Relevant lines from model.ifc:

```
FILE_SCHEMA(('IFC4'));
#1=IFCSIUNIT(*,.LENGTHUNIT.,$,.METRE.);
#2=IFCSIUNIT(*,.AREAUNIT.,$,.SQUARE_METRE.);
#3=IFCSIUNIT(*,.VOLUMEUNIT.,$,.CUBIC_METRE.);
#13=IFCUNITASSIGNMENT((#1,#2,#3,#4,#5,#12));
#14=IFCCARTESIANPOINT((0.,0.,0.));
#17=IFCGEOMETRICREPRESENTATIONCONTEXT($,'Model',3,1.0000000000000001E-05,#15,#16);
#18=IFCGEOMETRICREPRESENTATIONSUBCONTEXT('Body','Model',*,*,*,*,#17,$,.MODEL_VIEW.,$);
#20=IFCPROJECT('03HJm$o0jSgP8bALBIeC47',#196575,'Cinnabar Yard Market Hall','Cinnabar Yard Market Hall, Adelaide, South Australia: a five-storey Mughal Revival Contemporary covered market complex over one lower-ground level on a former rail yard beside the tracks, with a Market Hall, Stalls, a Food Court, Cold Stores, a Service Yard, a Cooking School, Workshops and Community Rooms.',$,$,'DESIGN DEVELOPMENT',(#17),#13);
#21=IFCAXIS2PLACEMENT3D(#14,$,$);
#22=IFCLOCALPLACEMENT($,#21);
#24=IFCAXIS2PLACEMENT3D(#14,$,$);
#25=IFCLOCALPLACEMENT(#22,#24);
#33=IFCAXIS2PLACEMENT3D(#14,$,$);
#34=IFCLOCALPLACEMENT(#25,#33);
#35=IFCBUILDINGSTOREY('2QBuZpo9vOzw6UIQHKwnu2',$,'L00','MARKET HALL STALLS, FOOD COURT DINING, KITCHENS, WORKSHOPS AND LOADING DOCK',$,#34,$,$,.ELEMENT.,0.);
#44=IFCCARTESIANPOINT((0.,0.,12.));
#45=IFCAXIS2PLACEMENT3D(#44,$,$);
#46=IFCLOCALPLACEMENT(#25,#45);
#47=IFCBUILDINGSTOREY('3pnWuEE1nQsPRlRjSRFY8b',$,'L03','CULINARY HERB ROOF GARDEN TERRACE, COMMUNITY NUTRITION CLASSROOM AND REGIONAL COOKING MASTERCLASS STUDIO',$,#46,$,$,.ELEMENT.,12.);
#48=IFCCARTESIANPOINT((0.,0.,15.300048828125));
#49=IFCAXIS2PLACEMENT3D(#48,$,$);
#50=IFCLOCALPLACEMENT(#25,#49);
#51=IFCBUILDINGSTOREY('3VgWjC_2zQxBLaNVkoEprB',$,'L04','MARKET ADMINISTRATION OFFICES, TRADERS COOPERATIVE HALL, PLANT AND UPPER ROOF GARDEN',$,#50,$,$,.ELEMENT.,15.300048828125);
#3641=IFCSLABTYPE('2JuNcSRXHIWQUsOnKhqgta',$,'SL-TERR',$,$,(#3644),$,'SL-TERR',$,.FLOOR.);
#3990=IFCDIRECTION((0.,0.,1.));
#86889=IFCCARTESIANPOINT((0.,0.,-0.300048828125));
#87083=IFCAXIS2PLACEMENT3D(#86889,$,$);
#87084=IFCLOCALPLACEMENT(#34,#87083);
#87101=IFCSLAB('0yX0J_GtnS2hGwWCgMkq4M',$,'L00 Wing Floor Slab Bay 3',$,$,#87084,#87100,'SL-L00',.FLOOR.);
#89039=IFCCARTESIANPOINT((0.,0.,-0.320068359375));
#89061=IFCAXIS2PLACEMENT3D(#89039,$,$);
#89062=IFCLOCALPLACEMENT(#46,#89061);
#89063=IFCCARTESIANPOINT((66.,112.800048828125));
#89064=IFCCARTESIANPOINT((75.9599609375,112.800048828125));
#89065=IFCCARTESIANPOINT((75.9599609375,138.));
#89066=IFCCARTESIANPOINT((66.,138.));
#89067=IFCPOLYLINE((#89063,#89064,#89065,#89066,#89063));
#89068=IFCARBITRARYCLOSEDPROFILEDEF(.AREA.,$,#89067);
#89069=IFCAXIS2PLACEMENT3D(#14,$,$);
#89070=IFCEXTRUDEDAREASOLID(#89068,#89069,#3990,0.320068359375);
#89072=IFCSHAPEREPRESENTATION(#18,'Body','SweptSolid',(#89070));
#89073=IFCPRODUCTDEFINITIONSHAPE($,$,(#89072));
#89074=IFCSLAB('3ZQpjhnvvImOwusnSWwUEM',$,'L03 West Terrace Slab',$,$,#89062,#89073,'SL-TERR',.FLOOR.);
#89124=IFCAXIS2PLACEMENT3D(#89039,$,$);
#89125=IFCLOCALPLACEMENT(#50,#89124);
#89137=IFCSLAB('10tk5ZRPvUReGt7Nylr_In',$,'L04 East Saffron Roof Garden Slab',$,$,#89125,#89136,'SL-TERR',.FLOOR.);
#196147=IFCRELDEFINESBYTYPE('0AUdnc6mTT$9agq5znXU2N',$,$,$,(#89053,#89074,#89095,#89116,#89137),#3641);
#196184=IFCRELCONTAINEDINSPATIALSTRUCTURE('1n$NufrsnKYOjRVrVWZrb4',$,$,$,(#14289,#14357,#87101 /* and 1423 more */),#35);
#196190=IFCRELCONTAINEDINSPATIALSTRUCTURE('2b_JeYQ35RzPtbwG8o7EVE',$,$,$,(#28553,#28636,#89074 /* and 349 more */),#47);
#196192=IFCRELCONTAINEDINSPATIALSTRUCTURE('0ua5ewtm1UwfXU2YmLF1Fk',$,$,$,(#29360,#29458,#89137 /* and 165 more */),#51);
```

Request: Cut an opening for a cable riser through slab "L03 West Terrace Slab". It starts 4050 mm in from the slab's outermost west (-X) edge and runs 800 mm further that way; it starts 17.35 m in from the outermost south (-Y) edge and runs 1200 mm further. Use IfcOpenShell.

```python
import numpy as np
import ifcopenshell
import ifcopenshell.api.feature
import ifcopenshell.api.geometry
import ifcopenshell.api.root
import ifcopenshell.geom
import ifcopenshell.util.placement
import ifcopenshell.util.representation
import ifcopenshell.util.shape
import ifcopenshell.util.unit

model = ifcopenshell.open("model.ifc")
unit_scale = ifcopenshell.util.unit.calculate_unit_scale(model)
settings = ifcopenshell.geom.settings()


def volume(element):
    """Net volume in cubic metres, openings subtracted."""
    shape = ifcopenshell.geom.create_shape(settings, element)
    return ifcopenshell.util.shape.get_volume(shape.geometry)


slab = model.by_id(89074)
before = volume(slab)

# Extent in the slab's own axes, in metres. The edges named are its -X and -Y sides.
slab_shape = ifcopenshell.geom.create_shape(settings, slab)
vertices = ifcopenshell.util.shape.get_vertices(slab_shape.geometry)
x_min, y_min, bottom = vertices.min(axis=0)
top = vertices[:, 2].max()

opening = ifcopenshell.api.root.create_entity(model, ifc_class="IfcOpeningElement", name="Cable riser opening", predefined_type="OPENING")
context = ifcopenshell.util.representation.get_context(model, "Model", "Body", "MODEL_VIEW")
width, depth = 0.8, 1.2
outline = [(0.0, 0.0), (width, 0.0), (width, depth), (0.0, depth), (0.0, 0.0)]
# Overshoot both faces by 50 mm so the cut is clean.
shape = ifcopenshell.api.geometry.add_slab_representation(
    model, context=context, depth=top - bottom + 0.1, polyline=outline
)
ifcopenshell.api.geometry.assign_representation(model, product=opening, representation=shape)

matrix = ifcopenshell.util.placement.get_local_placement(slab.ObjectPlacement)
matrix[:, 3] = matrix @ np.append(np.array([x_min + 4.05, y_min + 17.35, bottom - 0.05]) / unit_scale, 1.0)
ifcopenshell.api.geometry.edit_object_placement(model, product=opening, matrix=matrix, is_si=False)
ifcopenshell.api.feature.add_feature(model, feature=opening, element=slab)

after = volume(slab)

print(f"slab volume {before:.3f} -> {after:.3f} m3")

model.write("model_edited.ifc")
```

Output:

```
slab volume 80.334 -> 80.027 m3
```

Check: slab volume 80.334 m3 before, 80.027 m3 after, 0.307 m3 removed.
